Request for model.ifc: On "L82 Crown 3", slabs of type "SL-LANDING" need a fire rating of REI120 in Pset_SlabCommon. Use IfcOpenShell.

First a look at what the model holds.

```python
import ifcopenshell
import ifcopenshell.util.element

model = ifcopenshell.open("model.ifc")
print(model.schema)
storey = next(s for s in model.by_type("IfcBuildingStorey") if s.Name == "L82 Crown 3")
slabs = [e for e in ifcopenshell.util.element.get_decomposition(storey) if e.is_a("IfcSlab")]
seen = {}
for e in slabs:
    element_type = ifcopenshell.util.element.get_type(e)
    key = (element_type.Name if element_type != e and element_type else None, ifcopenshell.util.element.get_pset(e, "Pset_SlabCommon", "FireRating"))
    seen[key] = seen.get(key, 0) + 1
for (name, value), count in sorted(seen.items(), key=str):
    print(count, "x", name, "|", value)
```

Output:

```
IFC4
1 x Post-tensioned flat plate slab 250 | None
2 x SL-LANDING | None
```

```python
import ifcopenshell
import ifcopenshell.api.pset
import ifcopenshell.util.element

model = ifcopenshell.open("model.ifc")

storey = next(s for s in model.by_type("IfcBuildingStorey") if s.Name == "L82 Crown 3")
slabs = [e for e in ifcopenshell.util.element.get_decomposition(storey) if e.is_a("IfcSlab")]

count = 0
for e in slabs:
    element_type = ifcopenshell.util.element.get_type(e)
    if element_type in (None, e) or element_type.Name != "SL-LANDING":
        continue
    found = ifcopenshell.util.element.get_pset(e, "Pset_SlabCommon", should_inherit=False)
    if found:
        pset = model.by_id(found["id"])
        if len(ifcopenshell.util.element.get_elements_by_pset(pset)) > 1:
            pset = ifcopenshell.api.pset.unshare_pset(model, products=[e], pset=pset)[0]
    else:
        pset = ifcopenshell.api.pset.add_pset(model, product=e, name="Pset_SlabCommon")
    ifcopenshell.api.pset.edit_pset(model, pset=pset, properties={"FireRating": "REI120"})
    count += 1

print(count, "slabs updated")

model.write("model-out.ifc")
```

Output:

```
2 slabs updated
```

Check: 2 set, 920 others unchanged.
